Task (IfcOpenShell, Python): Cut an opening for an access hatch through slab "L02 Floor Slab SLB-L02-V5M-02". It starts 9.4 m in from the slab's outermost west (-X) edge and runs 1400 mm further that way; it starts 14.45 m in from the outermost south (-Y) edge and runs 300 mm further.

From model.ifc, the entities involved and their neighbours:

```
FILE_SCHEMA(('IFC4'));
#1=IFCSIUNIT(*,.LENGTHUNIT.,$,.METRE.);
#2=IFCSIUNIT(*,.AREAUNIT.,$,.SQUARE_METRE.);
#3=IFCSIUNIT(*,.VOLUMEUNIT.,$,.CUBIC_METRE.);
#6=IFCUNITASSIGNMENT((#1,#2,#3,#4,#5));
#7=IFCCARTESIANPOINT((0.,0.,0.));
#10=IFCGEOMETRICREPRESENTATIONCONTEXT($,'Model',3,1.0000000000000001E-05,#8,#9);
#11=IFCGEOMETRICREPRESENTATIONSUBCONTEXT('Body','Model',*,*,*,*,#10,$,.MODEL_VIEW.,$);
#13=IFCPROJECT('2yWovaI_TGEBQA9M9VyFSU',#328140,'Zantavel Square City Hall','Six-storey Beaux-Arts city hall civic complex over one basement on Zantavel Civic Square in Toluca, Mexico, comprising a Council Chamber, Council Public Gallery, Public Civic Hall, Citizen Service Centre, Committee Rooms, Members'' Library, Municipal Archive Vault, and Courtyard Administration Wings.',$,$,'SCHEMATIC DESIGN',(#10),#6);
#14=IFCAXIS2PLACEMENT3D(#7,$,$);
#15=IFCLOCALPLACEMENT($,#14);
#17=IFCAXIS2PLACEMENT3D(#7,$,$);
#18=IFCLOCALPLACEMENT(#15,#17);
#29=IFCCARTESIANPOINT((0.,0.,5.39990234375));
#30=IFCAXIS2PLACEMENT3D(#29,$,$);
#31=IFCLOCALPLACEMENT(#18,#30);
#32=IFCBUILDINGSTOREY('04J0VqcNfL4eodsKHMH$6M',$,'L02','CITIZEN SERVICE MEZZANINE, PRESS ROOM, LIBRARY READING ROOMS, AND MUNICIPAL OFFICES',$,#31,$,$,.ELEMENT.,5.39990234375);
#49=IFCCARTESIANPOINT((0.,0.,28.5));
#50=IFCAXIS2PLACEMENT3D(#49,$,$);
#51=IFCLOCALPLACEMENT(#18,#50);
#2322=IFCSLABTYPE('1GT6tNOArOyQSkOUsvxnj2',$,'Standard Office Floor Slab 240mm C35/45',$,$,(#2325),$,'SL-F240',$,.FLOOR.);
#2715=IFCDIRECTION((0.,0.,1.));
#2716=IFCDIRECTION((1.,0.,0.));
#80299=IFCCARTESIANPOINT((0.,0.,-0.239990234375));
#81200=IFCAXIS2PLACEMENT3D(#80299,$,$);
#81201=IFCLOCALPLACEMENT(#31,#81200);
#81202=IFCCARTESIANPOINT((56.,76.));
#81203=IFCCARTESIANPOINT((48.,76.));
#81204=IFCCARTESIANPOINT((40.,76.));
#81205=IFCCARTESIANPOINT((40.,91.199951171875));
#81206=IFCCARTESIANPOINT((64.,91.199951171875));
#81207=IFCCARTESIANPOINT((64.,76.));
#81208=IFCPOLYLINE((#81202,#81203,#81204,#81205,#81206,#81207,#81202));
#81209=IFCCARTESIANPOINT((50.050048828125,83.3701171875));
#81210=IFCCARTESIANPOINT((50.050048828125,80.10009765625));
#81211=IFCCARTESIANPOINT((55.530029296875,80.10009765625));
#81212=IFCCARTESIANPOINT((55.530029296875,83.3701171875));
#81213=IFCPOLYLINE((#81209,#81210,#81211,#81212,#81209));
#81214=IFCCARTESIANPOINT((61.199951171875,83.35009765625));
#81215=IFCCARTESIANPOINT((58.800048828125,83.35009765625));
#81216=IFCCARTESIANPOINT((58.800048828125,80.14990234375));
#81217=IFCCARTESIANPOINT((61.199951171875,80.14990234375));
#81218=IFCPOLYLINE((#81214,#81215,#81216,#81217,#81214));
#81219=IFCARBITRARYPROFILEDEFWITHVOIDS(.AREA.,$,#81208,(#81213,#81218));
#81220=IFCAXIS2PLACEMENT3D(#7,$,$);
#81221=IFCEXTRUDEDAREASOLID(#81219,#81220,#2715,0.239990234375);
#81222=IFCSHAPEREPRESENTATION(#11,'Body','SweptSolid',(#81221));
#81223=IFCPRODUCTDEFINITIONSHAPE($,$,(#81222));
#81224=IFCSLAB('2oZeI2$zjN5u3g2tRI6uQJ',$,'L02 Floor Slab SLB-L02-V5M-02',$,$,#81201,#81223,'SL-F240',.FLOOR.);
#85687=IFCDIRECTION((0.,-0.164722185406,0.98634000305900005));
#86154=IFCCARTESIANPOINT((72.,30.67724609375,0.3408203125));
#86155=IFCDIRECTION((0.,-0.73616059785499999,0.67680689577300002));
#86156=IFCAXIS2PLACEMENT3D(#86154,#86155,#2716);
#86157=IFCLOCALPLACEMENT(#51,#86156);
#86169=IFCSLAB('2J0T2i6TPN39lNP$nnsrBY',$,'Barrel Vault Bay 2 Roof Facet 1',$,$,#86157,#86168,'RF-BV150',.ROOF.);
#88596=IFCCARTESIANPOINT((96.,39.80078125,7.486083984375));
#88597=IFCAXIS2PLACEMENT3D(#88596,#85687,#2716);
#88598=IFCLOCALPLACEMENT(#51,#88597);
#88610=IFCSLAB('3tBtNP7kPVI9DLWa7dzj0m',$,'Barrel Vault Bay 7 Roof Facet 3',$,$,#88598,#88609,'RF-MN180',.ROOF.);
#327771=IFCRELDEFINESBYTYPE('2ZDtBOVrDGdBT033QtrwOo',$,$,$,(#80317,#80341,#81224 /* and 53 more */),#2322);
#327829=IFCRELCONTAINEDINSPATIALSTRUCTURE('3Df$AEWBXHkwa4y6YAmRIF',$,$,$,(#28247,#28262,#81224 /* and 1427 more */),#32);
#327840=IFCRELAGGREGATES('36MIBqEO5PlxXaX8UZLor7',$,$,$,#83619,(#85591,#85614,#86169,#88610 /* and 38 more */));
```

```python
import numpy as np
import ifcopenshell
import ifcopenshell.api.feature
import ifcopenshell.api.geometry
import ifcopenshell.api.root
import ifcopenshell.geom
import ifcopenshell.util.placement
import ifcopenshell.util.representation
import ifcopenshell.util.shape
import ifcopenshell.util.unit

model = ifcopenshell.open("model.ifc")
unit_scale = ifcopenshell.util.unit.calculate_unit_scale(model)
settings = ifcopenshell.geom.settings()


def volume(element):
    """Net volume in cubic metres, openings subtracted."""
    shape = ifcopenshell.geom.create_shape(settings, element)
    return ifcopenshell.util.shape.get_volume(shape.geometry)


slab = model.by_id(81224)
before = volume(slab)

# Extent in the slab's own axes, in metres. The edges named are its -X and -Y sides.
slab_shape = ifcopenshell.geom.create_shape(settings, slab)
vertices = ifcopenshell.util.shape.get_vertices(slab_shape.geometry)
x_min, y_min, bottom = vertices.min(axis=0)
top = vertices[:, 2].max()

opening = ifcopenshell.api.root.create_entity(model, ifc_class="IfcOpeningElement", name="Access hatch opening", predefined_type="OPENING")
context = ifcopenshell.util.representation.get_context(model, "Model", "Body", "MODEL_VIEW")
width, depth = 1.4, 0.3
outline = [(0.0, 0.0), (width, 0.0), (width, depth), (0.0, depth), (0.0, 0.0)]
# Overshoot both faces by 50 mm so the cut is clean.
shape = ifcopenshell.api.geometry.add_slab_representation(
    model, context=context, depth=top - bottom + 0.1, polyline=outline
)
ifcopenshell.api.geometry.assign_representation(model, product=opening, representation=shape)

matrix = ifcopenshell.util.placement.get_local_placement(slab.ObjectPlacement)
matrix[:, 3] = matrix @ np.append(np.array([x_min + 9.4, y_min + 14.45, bottom - 0.05]) / unit_scale, 1.0)
ifcopenshell.api.geometry.edit_object_placement(model, product=opening, matrix=matrix, is_si=False)
ifcopenshell.api.feature.add_feature(model, feature=opening, element=slab)

after = volume(slab)

print(f"slab volume {before:.3f} -> {after:.3f} m3")

model.write("model_v2.ifc")
```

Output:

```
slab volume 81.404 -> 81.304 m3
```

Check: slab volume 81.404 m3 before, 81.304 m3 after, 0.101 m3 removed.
